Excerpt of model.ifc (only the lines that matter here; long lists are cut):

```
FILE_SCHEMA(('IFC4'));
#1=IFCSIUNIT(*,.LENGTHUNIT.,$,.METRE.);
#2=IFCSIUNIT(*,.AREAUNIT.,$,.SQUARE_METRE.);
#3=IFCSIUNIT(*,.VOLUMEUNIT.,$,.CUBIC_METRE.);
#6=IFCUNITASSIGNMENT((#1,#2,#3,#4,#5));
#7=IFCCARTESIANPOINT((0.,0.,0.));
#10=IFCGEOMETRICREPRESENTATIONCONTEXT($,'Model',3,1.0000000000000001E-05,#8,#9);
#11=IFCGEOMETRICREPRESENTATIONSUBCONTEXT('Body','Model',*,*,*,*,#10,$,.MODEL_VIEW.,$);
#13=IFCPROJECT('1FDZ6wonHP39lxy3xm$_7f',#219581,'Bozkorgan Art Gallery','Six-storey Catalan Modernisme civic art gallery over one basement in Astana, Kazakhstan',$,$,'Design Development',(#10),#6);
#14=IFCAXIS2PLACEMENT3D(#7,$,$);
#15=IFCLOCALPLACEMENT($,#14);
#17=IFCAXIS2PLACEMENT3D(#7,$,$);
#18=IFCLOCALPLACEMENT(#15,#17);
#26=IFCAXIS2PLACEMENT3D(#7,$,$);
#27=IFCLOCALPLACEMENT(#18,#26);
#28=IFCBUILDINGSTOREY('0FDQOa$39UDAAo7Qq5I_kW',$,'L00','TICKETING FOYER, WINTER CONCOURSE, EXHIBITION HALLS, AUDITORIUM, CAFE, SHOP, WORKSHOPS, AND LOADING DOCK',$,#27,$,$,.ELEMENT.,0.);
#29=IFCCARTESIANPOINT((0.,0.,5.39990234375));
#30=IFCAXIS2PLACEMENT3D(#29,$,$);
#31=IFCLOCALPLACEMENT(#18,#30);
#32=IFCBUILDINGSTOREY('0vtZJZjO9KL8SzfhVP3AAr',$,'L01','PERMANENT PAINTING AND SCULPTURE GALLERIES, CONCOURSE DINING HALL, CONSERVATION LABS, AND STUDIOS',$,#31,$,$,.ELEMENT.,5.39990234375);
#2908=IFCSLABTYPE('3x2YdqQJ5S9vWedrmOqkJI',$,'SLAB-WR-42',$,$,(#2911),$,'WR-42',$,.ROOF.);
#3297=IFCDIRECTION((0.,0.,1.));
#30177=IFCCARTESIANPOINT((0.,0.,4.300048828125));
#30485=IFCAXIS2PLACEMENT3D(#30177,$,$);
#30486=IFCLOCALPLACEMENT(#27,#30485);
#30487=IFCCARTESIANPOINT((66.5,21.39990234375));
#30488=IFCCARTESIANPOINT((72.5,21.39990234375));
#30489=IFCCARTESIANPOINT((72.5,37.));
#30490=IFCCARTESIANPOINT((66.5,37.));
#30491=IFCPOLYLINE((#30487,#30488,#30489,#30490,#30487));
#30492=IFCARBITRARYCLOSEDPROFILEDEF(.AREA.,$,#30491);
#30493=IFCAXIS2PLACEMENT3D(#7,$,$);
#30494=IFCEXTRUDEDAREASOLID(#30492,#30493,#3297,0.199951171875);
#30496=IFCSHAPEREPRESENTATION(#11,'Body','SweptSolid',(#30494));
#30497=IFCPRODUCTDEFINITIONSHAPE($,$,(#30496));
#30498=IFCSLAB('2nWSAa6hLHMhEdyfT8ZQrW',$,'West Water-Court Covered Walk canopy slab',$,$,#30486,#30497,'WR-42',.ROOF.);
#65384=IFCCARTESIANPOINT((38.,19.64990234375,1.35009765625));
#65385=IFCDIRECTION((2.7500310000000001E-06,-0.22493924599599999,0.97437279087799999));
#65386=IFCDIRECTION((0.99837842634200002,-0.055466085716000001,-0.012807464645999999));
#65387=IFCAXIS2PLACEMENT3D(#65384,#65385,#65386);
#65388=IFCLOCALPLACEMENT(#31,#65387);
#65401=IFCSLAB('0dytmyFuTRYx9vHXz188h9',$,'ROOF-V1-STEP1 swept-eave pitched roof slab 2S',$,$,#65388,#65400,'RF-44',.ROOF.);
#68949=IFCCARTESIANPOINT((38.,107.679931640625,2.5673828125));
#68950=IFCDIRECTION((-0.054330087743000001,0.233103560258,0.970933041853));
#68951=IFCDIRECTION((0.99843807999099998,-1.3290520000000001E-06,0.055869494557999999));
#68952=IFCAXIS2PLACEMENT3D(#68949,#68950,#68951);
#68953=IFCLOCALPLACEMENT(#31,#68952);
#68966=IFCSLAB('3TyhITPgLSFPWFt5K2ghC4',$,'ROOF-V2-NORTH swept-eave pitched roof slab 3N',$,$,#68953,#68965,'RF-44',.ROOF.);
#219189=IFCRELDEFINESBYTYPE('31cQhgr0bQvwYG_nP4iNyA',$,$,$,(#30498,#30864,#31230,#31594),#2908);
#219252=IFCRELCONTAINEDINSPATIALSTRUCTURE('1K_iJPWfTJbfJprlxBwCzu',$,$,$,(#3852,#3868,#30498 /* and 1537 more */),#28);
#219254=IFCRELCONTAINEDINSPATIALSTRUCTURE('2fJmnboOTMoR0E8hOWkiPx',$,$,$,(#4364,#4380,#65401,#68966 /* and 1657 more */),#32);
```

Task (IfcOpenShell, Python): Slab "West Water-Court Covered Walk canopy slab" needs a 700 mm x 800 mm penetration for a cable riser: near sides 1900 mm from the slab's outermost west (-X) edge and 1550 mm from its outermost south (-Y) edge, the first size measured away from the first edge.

```python
import numpy as np
import ifcopenshell
import ifcopenshell.api.feature
import ifcopenshell.api.geometry
import ifcopenshell.api.root
import ifcopenshell.geom
import ifcopenshell.util.placement
import ifcopenshell.util.representation
import ifcopenshell.util.shape
import ifcopenshell.util.unit

model = ifcopenshell.open("model.ifc")
unit_scale = ifcopenshell.util.unit.calculate_unit_scale(model)
settings = ifcopenshell.geom.settings()


def volume(element):
    """Net volume in cubic metres, openings subtracted."""
    shape = ifcopenshell.geom.create_shape(settings, element)
    return ifcopenshell.util.shape.get_volume(shape.geometry)


slab = model.by_guid("2nWSAa6hLHMhEdyfT8ZQrW")
before = volume(slab)

# Extent in the slab's own axes, in metres. The edges named are its -X and -Y sides.
slab_shape = ifcopenshell.geom.create_shape(settings, slab)
vertices = ifcopenshell.util.shape.get_vertices(slab_shape.geometry)
x_min, y_min, bottom = vertices.min(axis=0)
top = vertices[:, 2].max()

opening = ifcopenshell.api.root.create_entity(model, ifc_class="IfcOpeningElement", name="Cable riser opening", predefined_type="OPENING")
context = ifcopenshell.util.representation.get_context(model, "Model", "Body", "MODEL_VIEW")
width, depth = 0.7, 0.8
outline = [(0.0, 0.0), (width, 0.0), (width, depth), (0.0, depth), (0.0, 0.0)]
# Overshoot both faces by 50 mm so the cut is clean.
shape = ifcopenshell.api.geometry.add_slab_representation(
    model, context=context, depth=top - bottom + 0.1, polyline=outline
)
ifcopenshell.api.geometry.assign_representation(model, product=opening, representation=shape)

matrix = ifcopenshell.util.placement.get_local_placement(slab.ObjectPlacement)
matrix[:, 3] = matrix @ np.append(np.array([x_min + 1.9, y_min + 1.55, bottom - 0.05]) / unit_scale, 1.0)
ifcopenshell.api.geometry.edit_object_placement(model, product=opening, matrix=matrix, is_si=False)
ifcopenshell.api.feature.add_feature(model, feature=opening, element=slab)

after = volume(slab)

print(f"slab volume {before:.3f} -> {after:.3f} m3")

model.write("model-out.ifc")
```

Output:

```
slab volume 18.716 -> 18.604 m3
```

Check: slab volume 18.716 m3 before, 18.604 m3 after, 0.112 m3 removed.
